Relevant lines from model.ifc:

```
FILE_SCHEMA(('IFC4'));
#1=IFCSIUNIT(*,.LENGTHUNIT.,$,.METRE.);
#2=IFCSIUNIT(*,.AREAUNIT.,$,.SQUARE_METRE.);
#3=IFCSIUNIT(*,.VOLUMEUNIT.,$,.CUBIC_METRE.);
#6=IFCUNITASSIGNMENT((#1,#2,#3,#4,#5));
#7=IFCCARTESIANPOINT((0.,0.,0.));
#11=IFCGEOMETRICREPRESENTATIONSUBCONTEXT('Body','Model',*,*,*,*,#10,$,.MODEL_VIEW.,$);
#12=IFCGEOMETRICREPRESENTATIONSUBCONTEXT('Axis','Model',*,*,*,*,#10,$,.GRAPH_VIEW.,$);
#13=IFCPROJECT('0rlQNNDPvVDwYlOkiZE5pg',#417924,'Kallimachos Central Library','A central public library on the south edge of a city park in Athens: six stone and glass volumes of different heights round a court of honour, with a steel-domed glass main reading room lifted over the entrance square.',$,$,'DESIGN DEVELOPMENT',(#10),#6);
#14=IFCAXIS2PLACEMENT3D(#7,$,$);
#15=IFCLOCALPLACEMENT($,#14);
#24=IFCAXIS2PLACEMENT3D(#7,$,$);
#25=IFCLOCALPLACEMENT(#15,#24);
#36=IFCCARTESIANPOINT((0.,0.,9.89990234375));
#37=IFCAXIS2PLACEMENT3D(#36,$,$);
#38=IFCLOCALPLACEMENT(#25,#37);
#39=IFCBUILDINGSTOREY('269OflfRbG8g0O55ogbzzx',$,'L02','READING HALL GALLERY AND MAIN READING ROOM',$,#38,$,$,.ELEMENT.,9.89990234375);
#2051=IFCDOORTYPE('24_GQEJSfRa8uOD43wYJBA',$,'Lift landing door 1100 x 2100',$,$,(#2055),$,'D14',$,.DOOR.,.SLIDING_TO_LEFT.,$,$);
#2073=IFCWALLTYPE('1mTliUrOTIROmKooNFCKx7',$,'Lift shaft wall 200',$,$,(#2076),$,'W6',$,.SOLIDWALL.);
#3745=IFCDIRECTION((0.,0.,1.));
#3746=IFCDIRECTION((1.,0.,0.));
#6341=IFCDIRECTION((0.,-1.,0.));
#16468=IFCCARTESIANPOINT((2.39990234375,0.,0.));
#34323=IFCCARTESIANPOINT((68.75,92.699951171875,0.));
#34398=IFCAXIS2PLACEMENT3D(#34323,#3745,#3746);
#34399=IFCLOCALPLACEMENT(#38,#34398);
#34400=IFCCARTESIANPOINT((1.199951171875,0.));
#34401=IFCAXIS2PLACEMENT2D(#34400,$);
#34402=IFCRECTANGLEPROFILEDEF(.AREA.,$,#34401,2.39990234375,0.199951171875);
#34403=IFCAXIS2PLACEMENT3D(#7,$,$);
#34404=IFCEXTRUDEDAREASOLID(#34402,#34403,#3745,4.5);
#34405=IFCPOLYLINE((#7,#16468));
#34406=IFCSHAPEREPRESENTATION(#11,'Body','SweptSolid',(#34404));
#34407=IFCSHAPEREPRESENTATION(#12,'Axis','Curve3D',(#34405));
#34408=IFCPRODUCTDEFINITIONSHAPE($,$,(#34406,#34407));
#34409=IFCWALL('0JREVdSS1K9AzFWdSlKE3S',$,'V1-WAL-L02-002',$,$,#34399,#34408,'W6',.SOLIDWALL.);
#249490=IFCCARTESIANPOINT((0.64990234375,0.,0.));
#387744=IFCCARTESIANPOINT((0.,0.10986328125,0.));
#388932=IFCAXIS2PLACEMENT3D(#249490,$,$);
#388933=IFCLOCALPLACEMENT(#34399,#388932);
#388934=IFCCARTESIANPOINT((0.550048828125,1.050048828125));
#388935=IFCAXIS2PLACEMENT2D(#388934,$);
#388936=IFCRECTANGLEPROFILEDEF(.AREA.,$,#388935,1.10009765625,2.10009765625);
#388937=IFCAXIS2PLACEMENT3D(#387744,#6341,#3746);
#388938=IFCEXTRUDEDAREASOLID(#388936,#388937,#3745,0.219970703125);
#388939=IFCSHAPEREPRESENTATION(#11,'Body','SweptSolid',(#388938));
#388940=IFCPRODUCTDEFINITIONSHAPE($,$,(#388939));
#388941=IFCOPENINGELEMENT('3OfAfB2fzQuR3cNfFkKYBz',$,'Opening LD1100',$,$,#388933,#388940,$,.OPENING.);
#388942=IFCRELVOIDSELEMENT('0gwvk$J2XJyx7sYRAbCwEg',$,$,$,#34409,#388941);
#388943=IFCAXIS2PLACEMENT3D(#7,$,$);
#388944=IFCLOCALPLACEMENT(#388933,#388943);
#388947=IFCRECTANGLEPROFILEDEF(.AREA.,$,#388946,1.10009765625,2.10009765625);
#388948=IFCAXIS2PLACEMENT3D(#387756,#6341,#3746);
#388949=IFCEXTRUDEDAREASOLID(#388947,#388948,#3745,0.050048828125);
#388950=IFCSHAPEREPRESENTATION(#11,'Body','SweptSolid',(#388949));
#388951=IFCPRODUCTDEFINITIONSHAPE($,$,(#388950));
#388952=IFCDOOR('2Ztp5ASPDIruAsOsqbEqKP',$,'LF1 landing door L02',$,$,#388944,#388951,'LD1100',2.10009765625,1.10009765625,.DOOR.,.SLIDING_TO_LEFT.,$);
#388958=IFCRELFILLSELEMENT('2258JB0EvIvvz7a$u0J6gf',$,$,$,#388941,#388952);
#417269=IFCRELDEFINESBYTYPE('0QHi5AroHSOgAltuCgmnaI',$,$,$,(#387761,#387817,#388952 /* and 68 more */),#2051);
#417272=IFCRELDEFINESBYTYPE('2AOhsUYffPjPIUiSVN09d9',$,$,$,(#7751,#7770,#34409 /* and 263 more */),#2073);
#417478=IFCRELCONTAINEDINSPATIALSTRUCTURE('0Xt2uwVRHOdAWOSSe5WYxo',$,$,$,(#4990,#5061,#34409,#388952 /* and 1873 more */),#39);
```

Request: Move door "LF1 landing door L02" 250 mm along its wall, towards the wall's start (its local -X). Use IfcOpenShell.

```python
import ifcopenshell
import ifcopenshell.api.geometry
import ifcopenshell.util.placement
import ifcopenshell.util.unit

model = ifcopenshell.open("model.ifc")
unit_scale = ifcopenshell.util.unit.calculate_unit_scale(model)

door = model.by_guid("2Ztp5ASPDIruAsOsqbEqKP")
opening = door.FillsVoids[0].RelatingOpeningElement
wall = opening.VoidsElements[0].RelatingBuildingElement

wall_matrix = ifcopenshell.util.placement.get_local_placement(wall.ObjectPlacement)
shift = wall_matrix[:3, 0] * -0.25 / unit_scale
before = ifcopenshell.util.placement.get_local_placement(door.ObjectPlacement)[:3, 3].copy()

# The door is placed relative to its opening, so it follows when the opening moves.
matrix = ifcopenshell.util.placement.get_local_placement(opening.ObjectPlacement)
matrix[:3, 3] += shift
ifcopenshell.api.geometry.edit_object_placement(
    model, product=opening, matrix=matrix, is_si=False, should_transform_children=True
)

after = ifcopenshell.util.placement.get_local_placement(door.ObjectPlacement)[:3, 3]
print("door moved by", (after - before).round(3) + 0.0)

model.write("model_updated.ifc")
```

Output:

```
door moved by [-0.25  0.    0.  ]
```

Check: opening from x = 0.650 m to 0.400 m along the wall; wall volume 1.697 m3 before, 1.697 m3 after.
